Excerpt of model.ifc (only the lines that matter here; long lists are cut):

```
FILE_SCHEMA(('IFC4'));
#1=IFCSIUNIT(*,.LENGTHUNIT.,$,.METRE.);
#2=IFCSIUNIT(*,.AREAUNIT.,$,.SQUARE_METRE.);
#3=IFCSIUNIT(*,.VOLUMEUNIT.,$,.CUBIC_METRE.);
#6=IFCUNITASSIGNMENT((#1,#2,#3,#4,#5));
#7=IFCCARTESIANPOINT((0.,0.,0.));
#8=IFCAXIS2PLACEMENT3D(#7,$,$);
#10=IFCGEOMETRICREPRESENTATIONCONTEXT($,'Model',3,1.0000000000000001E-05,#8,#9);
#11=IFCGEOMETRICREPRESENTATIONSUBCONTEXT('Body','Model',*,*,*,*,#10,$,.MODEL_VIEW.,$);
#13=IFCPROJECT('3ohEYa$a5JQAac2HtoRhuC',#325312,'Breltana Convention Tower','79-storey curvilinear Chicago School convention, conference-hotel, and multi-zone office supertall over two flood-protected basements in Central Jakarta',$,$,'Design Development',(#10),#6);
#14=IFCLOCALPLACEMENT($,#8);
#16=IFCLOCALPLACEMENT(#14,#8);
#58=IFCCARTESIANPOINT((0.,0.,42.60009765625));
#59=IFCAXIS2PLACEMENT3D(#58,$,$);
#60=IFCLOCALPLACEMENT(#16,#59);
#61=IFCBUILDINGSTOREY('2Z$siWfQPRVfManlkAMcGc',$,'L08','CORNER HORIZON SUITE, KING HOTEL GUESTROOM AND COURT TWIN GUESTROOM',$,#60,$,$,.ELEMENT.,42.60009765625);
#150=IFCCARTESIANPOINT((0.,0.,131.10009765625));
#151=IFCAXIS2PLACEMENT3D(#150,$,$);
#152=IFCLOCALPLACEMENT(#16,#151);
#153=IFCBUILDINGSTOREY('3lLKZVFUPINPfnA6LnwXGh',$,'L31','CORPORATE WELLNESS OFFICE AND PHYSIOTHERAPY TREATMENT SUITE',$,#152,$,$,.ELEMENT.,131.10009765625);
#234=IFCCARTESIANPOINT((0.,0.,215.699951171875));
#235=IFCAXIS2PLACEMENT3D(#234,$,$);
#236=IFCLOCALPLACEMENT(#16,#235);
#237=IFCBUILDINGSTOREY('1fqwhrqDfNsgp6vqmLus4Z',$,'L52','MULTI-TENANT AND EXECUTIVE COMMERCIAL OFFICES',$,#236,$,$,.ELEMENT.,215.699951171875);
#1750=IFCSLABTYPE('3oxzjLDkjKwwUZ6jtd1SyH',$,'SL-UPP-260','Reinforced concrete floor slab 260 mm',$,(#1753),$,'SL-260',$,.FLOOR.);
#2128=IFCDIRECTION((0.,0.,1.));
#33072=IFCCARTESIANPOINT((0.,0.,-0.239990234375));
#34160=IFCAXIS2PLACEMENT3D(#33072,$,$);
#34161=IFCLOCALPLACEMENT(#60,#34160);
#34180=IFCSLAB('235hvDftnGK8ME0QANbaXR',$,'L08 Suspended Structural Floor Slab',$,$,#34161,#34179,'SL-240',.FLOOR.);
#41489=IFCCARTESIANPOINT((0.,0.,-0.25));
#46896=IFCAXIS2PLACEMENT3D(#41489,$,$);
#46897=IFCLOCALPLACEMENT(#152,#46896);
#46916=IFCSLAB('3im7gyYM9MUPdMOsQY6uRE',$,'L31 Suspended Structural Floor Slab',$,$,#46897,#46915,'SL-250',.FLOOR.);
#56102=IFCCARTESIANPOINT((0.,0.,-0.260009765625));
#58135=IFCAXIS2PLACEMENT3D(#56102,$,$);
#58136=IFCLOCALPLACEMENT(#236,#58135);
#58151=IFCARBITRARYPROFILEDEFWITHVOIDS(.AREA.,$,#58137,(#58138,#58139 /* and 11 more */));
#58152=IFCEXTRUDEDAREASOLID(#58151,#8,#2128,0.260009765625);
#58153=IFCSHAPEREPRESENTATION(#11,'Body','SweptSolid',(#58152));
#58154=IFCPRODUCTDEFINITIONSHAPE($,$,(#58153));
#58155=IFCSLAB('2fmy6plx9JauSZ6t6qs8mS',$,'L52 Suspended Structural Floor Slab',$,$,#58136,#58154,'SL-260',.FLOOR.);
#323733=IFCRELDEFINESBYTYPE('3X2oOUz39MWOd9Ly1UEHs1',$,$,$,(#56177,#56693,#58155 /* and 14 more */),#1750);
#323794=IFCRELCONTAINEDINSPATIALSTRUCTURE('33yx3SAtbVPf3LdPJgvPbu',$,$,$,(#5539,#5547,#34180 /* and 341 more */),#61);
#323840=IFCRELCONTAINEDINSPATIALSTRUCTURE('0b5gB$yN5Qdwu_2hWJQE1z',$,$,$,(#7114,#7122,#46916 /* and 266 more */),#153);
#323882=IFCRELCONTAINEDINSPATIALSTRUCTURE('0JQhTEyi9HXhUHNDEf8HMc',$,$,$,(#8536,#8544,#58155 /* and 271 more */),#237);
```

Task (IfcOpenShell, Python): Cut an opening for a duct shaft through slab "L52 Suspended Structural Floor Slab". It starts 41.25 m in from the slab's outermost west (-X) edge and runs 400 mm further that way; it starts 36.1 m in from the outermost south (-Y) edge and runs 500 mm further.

```python
import numpy as np
import ifcopenshell
import ifcopenshell.api.feature
import ifcopenshell.api.geometry
import ifcopenshell.api.root
import ifcopenshell.geom
import ifcopenshell.util.placement
import ifcopenshell.util.representation
import ifcopenshell.util.shape
import ifcopenshell.util.unit

model = ifcopenshell.open("model.ifc")
unit_scale = ifcopenshell.util.unit.calculate_unit_scale(model)
settings = ifcopenshell.geom.settings()


def volume(element):
    """Net volume in cubic metres, openings subtracted."""
    shape = ifcopenshell.geom.create_shape(settings, element)
    return ifcopenshell.util.shape.get_volume(shape.geometry)


slab = model.by_id(58155)
before = volume(slab)

# Extent in the slab's own axes, in metres. The edges named are its -X and -Y sides.
slab_shape = ifcopenshell.geom.create_shape(settings, slab)
vertices = ifcopenshell.util.shape.get_vertices(slab_shape.geometry)
x_min, y_min, bottom = vertices.min(axis=0)
top = vertices[:, 2].max()

opening = ifcopenshell.api.root.create_entity(model, ifc_class="IfcOpeningElement", name="Duct shaft opening", predefined_type="OPENING")
context = ifcopenshell.util.representation.get_context(model, "Model", "Body", "MODEL_VIEW")
width, depth = 0.4, 0.5
outline = [(0.0, 0.0), (width, 0.0), (width, depth), (0.0, depth), (0.0, 0.0)]
# Overshoot both faces by 50 mm so the cut is clean.
shape = ifcopenshell.api.geometry.add_slab_representation(
    model, context=context, depth=top - bottom + 0.1, polyline=outline
)
ifcopenshell.api.geometry.assign_representation(model, product=opening, representation=shape)

matrix = ifcopenshell.util.placement.get_local_placement(slab.ObjectPlacement)
matrix[:, 3] = matrix @ np.append(np.array([x_min + 41.25, y_min + 36.1, bottom - 0.05]) / unit_scale, 1.0)
ifcopenshell.api.geometry.edit_object_placement(model, product=opening, matrix=matrix, is_si=False)
ifcopenshell.api.feature.add_feature(model, feature=opening, element=slab)

after = volume(slab)

print(f"slab volume {before:.3f} -> {after:.3f} m3")

model.write("model-out.ifc")
```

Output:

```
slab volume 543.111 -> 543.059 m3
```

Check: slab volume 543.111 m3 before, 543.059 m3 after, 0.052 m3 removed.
